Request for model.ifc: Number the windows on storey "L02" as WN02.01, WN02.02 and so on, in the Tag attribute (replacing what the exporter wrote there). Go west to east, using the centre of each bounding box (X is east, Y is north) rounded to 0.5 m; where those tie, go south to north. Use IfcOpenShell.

First a look at what the model holds.

```python
import ifcopenshell
import ifcopenshell.util.element
import ifcopenshell.util.placement

model = ifcopenshell.open("model.ifc")
print(model.schema)
storey = next(s for s in model.by_type("IfcBuildingStorey") if s.Name == "L02")
windows = [e for e in ifcopenshell.util.element.get_decomposition(storey) if e.is_a("IfcWindow")]
for e in sorted(windows, key=lambda e: e.id()):
    origin = ifcopenshell.util.placement.get_local_placement(e.ObjectPlacement)[:3, 3]
    print(e.id(), e.Tag, e.Name, origin.round(2) + 0.0, sep=" | ")
```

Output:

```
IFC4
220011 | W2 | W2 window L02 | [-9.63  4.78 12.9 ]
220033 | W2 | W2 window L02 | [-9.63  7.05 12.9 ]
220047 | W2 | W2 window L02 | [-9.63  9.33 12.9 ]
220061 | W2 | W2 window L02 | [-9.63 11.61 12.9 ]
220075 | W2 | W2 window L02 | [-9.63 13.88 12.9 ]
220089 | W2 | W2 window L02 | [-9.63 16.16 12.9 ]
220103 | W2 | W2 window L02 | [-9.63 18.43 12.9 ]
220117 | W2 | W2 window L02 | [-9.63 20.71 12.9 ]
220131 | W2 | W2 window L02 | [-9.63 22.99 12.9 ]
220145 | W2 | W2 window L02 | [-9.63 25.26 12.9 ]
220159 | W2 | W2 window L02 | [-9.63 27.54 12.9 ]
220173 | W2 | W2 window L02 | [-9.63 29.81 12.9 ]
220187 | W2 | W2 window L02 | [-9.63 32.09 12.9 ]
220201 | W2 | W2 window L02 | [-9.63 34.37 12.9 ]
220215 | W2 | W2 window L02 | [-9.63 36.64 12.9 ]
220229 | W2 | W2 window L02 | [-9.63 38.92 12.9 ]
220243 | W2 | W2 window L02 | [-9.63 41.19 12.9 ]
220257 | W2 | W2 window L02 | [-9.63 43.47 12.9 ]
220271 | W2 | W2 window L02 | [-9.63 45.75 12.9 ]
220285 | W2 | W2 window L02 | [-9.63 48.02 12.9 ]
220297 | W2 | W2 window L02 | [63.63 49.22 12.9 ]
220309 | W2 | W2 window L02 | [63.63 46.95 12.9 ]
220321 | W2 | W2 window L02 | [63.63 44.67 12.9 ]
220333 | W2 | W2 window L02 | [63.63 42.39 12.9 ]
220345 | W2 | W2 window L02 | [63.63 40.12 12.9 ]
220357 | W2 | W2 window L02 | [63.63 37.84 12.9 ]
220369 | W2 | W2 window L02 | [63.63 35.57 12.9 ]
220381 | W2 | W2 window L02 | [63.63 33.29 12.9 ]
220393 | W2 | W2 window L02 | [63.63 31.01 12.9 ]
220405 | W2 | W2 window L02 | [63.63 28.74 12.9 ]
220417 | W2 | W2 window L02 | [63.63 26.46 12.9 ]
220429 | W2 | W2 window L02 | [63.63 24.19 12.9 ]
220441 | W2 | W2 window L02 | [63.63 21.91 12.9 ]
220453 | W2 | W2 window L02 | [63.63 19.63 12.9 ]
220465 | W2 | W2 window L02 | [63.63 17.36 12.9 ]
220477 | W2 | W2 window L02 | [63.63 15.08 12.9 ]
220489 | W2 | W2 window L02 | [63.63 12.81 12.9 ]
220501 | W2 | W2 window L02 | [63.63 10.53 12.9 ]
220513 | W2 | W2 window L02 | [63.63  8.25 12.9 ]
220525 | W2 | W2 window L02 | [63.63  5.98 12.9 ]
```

```python
import ifcopenshell
import ifcopenshell.geom
import ifcopenshell.util.element
import ifcopenshell.util.shape

model = ifcopenshell.open("model.ifc")
settings = ifcopenshell.geom.settings()
settings.set("use-world-coords", True)


def centre(element):
    shape = ifcopenshell.geom.create_shape(settings, element)
    return ifcopenshell.util.shape.get_bbox_centroid(shape.geometry)


storey = next(s for s in model.by_type("IfcBuildingStorey") if s.Name == "L02")
windows = [e for e in ifcopenshell.util.element.get_decomposition(storey) if e.is_a("IfcWindow")]

# Insertion points can sit at a corner or the storey origin, so sort by the geometry (in metres).
centres = {e: centre(e) for e in windows}
windows.sort(key=lambda e: (round(centres[e][0] / 0.5), centres[e][1]))

for i, e in enumerate(windows, start=1):
    number = f"WN02.{i:02d}"
    e.Tag = number
    print(e.id(), number)

model.write("model-out.ifc")
```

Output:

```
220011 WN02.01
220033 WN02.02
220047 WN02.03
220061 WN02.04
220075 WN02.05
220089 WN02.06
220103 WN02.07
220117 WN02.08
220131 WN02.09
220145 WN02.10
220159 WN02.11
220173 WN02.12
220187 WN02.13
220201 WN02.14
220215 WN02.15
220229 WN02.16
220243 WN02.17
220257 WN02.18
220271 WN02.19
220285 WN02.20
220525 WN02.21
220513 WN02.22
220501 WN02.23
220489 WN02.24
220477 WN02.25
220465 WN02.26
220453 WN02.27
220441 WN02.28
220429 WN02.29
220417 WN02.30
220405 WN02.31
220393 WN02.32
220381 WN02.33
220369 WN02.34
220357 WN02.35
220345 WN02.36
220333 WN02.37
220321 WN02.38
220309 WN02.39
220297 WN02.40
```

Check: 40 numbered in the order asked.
